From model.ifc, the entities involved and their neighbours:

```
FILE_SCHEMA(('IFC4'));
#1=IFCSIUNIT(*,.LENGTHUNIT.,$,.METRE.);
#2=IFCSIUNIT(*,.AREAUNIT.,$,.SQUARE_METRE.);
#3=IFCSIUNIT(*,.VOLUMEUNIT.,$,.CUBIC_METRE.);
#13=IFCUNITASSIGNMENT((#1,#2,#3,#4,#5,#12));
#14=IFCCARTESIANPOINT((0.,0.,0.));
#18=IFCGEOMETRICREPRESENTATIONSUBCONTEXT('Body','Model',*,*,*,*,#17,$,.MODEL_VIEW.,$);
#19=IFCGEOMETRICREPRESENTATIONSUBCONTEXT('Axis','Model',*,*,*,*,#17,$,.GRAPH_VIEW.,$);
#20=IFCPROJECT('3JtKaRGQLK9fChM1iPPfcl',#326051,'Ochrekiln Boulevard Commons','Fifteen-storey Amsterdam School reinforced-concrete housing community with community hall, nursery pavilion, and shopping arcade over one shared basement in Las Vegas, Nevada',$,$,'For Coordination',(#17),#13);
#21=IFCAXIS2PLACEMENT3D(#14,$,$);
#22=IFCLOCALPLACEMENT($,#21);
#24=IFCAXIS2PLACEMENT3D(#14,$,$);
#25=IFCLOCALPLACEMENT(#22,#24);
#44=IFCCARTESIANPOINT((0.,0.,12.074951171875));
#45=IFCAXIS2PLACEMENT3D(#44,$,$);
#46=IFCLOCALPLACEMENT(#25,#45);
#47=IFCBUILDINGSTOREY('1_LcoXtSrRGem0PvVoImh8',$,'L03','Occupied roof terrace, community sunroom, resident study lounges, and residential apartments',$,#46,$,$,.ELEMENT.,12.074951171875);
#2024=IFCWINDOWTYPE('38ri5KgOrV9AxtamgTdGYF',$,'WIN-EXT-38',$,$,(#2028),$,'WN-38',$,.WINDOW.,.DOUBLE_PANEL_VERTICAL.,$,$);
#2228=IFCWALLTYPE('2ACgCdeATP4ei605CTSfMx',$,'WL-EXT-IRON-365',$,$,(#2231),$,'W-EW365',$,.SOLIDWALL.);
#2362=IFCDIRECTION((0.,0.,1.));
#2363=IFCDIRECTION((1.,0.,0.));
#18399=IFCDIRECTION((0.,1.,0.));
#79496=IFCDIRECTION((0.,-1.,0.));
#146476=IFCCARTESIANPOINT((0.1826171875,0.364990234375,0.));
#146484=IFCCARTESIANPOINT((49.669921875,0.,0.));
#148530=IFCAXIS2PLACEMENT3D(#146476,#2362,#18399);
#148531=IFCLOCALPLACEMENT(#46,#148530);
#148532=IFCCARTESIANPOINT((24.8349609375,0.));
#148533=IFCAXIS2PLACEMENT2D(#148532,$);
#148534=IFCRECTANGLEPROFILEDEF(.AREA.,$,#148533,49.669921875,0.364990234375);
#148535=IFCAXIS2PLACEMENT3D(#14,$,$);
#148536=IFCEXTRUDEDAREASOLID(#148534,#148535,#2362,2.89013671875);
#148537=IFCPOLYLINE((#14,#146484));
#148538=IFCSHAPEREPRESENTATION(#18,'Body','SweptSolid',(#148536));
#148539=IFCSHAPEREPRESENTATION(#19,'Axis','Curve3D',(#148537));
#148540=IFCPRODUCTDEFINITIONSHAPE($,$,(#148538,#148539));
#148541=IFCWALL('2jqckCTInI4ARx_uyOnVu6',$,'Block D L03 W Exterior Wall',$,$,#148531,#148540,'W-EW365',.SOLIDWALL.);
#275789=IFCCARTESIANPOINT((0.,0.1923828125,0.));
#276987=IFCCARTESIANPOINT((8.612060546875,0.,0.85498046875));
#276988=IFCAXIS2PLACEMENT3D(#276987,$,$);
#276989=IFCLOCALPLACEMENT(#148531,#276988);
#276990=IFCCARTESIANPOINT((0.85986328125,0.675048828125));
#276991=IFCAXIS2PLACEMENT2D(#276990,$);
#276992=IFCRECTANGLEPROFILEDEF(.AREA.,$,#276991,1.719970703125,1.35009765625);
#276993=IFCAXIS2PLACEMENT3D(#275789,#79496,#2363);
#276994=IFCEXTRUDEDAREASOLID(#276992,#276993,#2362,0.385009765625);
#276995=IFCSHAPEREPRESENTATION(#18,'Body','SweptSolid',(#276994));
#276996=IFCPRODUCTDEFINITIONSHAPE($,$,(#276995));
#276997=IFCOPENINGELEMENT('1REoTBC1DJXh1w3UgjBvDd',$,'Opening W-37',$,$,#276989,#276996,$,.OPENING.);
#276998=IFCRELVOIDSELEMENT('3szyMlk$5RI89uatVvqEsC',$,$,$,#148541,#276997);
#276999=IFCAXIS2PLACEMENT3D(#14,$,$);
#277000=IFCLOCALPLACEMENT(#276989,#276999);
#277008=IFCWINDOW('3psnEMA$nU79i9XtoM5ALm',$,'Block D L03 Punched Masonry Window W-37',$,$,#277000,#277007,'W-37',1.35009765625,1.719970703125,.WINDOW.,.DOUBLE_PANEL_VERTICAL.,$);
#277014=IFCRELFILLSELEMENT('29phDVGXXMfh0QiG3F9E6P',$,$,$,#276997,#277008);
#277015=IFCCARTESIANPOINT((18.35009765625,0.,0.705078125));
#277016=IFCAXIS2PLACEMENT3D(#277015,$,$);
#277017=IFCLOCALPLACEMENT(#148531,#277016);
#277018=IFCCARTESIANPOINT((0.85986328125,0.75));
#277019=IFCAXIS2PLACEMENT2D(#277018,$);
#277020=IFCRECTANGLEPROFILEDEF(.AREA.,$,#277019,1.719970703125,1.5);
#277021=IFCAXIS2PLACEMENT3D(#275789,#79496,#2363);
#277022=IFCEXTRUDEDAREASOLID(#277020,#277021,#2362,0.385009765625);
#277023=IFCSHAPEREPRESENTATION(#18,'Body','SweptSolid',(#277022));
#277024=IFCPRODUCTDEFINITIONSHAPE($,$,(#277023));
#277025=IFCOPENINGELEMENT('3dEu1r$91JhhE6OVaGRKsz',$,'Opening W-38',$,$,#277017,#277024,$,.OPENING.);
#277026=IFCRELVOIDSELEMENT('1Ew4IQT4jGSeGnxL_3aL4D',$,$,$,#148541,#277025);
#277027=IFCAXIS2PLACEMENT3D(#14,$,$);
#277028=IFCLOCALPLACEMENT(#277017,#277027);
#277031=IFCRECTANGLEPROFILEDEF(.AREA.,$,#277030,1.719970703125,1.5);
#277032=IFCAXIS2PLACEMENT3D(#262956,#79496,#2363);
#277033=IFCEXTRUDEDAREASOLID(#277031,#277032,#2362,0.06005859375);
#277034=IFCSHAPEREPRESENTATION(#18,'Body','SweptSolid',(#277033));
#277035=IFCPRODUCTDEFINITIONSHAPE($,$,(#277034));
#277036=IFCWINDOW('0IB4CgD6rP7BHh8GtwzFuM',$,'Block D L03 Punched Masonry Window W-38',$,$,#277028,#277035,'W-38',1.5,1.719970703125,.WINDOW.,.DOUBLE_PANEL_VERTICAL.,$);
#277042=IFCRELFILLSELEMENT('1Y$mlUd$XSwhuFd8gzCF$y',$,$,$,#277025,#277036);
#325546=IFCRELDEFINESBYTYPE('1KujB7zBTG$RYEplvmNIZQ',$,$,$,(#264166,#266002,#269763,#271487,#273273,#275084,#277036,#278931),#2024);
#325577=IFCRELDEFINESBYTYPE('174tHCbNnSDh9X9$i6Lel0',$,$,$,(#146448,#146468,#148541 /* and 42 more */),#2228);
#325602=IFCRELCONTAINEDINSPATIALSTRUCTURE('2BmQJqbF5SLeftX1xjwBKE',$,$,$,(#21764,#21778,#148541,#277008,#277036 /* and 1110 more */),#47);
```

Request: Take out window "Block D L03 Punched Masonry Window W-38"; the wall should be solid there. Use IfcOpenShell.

```python
import ifcopenshell
import ifcopenshell.api.feature
import ifcopenshell.api.root
import ifcopenshell.geom
import ifcopenshell.util.shape

model = ifcopenshell.open("model.ifc")
settings = ifcopenshell.geom.settings()


def volume(element):
    """Net volume in cubic metres, openings subtracted."""
    shape = ifcopenshell.geom.create_shape(settings, element)
    return ifcopenshell.util.shape.get_volume(shape.geometry)


window = model.by_guid("0IB4CgD6rP7BHh8GtwzFuM")
opening = window.FillsVoids[0].RelatingOpeningElement
wall = opening.VoidsElements[0].RelatingBuildingElement
before = volume(wall)

ifcopenshell.api.root.remove_product(model, product=window)
ifcopenshell.api.feature.remove_feature(model, feature=opening)

after = volume(wall)

print(f"wall volume {before:.3f} -> {after:.3f} m3")

model.write("model_rev.ifc")
```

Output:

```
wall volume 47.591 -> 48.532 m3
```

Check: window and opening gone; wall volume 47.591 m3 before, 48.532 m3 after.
